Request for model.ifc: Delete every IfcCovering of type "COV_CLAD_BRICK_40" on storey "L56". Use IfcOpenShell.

First a look at what the model holds.

```python
import ifcopenshell
import ifcopenshell.util.element

model = ifcopenshell.open("model.ifc")
print(model.schema)
storey = next(s for s in model.by_type("IfcBuildingStorey") if s.Name == "L56")
coverings = [e for e in ifcopenshell.util.element.get_decomposition(storey) if e.is_a("IfcCovering")]
seen = {}
for e in coverings:
    element_type = ifcopenshell.util.element.get_type(e)
    name = element_type.Name if element_type not in (None, e) else None
    seen[name] = seen.get(name, 0) + 1
for name, count in sorted(seen.items(), key=str):
    print(count, "x", name)
```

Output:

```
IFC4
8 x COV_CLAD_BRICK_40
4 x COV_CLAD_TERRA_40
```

```python
import ifcopenshell
import ifcopenshell.api.root
import ifcopenshell.util.element

model = ifcopenshell.open("model.ifc")

storey = next(s for s in model.by_type("IfcBuildingStorey") if s.Name == "L56")
coverings = [e for e in ifcopenshell.util.element.get_decomposition(storey) if e.is_a("IfcCovering")]
targets = [e for e in coverings if (t := ifcopenshell.util.element.get_type(e)) not in (None, e) and t.Name == "COV_CLAD_BRICK_40"]

for e in targets:
    ifcopenshell.api.root.remove_product(model, product=e)
print(len(targets), "removed")

model.write("model-out.ifc")
```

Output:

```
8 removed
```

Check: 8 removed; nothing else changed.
